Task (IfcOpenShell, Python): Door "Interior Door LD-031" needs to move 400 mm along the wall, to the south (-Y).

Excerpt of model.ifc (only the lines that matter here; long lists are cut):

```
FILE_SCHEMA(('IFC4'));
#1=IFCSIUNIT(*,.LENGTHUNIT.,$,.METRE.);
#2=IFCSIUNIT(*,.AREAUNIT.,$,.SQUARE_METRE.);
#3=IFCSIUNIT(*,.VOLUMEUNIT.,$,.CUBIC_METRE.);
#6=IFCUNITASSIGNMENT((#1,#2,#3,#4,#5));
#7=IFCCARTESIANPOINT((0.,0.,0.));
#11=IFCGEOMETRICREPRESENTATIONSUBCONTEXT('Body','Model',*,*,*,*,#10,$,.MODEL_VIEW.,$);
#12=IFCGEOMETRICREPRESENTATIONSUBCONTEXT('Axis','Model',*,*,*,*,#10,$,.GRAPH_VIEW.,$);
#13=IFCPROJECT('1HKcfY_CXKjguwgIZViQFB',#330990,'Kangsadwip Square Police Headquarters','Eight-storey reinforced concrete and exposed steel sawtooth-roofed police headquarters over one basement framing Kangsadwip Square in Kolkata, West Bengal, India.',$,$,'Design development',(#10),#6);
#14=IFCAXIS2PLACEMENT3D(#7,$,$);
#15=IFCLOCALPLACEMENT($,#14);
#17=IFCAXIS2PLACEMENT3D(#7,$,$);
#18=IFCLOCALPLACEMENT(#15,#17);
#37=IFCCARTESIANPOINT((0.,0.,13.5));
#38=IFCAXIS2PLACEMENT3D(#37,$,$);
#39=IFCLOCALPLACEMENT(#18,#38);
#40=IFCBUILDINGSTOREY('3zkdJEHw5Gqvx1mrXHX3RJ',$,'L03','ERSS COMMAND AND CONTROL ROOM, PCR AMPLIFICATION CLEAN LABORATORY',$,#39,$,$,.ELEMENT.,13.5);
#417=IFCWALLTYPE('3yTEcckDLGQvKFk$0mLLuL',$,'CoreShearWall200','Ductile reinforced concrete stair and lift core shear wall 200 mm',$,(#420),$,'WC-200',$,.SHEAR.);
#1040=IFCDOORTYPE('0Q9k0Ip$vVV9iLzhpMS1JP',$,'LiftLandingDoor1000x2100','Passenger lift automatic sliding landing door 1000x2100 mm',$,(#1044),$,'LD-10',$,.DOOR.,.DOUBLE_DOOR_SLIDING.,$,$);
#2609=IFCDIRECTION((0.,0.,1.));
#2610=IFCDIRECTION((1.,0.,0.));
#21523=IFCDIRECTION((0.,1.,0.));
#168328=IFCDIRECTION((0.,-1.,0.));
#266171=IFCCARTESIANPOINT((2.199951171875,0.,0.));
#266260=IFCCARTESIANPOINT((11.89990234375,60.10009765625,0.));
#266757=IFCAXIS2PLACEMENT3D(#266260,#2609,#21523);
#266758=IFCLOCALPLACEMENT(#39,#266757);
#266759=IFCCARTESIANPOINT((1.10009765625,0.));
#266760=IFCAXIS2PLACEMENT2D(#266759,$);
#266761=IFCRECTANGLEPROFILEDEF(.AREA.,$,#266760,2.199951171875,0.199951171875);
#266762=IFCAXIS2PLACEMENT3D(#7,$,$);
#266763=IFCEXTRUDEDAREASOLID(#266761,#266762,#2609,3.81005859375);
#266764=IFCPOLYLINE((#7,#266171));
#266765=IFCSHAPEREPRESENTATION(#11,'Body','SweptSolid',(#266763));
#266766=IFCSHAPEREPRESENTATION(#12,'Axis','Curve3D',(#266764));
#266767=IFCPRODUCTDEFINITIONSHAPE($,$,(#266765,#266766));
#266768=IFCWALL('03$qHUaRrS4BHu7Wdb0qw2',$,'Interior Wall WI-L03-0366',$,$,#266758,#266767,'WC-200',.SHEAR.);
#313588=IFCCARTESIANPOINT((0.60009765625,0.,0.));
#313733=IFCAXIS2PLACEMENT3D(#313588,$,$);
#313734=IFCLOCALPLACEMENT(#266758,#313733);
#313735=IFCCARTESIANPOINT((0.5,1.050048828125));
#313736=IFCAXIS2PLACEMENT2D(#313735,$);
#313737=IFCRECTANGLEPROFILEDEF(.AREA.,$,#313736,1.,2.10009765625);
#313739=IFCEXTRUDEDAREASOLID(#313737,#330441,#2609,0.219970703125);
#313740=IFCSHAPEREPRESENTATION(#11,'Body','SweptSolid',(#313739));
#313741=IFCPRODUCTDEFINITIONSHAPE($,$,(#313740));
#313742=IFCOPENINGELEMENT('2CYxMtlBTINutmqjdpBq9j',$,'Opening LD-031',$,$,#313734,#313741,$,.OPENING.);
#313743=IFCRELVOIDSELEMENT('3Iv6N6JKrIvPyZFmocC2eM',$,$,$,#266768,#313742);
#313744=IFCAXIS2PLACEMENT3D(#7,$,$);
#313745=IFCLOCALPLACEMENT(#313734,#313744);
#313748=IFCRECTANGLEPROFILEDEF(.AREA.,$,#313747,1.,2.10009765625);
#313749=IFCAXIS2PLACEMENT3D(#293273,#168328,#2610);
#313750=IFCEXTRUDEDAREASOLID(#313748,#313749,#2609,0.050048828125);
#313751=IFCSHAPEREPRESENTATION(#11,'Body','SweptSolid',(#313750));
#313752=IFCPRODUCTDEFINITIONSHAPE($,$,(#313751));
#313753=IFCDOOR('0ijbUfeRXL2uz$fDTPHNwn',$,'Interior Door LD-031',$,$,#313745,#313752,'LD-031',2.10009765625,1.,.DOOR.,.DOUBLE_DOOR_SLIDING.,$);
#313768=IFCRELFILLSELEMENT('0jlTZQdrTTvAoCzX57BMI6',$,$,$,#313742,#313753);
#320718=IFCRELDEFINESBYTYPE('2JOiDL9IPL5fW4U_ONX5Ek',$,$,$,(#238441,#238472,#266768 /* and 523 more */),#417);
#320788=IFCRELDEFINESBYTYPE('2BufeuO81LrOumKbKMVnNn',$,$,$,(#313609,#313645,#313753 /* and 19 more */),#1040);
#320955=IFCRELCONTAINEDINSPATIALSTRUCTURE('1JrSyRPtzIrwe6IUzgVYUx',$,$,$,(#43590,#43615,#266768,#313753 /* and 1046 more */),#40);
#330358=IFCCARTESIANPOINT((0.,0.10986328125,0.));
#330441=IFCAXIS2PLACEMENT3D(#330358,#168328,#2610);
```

```python
import ifcopenshell
import ifcopenshell.api.geometry
import ifcopenshell.util.placement
import ifcopenshell.util.unit

model = ifcopenshell.open("model.ifc")
unit_scale = ifcopenshell.util.unit.calculate_unit_scale(model)

door = model.by_guid("0ijbUfeRXL2uz$fDTPHNwn")
opening = door.FillsVoids[0].RelatingOpeningElement
wall = opening.VoidsElements[0].RelatingBuildingElement

wall_matrix = ifcopenshell.util.placement.get_local_placement(wall.ObjectPlacement)
shift = wall_matrix[:3, 0] * -0.4 / unit_scale
before = ifcopenshell.util.placement.get_local_placement(door.ObjectPlacement)[:3, 3].copy()

# The door is placed relative to its opening, so it follows when the opening moves.
matrix = ifcopenshell.util.placement.get_local_placement(opening.ObjectPlacement)
matrix[:3, 3] += shift
ifcopenshell.api.geometry.edit_object_placement(
    model, product=opening, matrix=matrix, is_si=False, should_transform_children=True
)

after = ifcopenshell.util.placement.get_local_placement(door.ObjectPlacement)[:3, 3]
print("door moved by", (after - before).round(3) + 0.0)

model.write("model_v2.ifc")
```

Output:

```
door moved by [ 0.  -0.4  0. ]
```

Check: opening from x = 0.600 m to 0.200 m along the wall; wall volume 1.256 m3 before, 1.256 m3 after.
